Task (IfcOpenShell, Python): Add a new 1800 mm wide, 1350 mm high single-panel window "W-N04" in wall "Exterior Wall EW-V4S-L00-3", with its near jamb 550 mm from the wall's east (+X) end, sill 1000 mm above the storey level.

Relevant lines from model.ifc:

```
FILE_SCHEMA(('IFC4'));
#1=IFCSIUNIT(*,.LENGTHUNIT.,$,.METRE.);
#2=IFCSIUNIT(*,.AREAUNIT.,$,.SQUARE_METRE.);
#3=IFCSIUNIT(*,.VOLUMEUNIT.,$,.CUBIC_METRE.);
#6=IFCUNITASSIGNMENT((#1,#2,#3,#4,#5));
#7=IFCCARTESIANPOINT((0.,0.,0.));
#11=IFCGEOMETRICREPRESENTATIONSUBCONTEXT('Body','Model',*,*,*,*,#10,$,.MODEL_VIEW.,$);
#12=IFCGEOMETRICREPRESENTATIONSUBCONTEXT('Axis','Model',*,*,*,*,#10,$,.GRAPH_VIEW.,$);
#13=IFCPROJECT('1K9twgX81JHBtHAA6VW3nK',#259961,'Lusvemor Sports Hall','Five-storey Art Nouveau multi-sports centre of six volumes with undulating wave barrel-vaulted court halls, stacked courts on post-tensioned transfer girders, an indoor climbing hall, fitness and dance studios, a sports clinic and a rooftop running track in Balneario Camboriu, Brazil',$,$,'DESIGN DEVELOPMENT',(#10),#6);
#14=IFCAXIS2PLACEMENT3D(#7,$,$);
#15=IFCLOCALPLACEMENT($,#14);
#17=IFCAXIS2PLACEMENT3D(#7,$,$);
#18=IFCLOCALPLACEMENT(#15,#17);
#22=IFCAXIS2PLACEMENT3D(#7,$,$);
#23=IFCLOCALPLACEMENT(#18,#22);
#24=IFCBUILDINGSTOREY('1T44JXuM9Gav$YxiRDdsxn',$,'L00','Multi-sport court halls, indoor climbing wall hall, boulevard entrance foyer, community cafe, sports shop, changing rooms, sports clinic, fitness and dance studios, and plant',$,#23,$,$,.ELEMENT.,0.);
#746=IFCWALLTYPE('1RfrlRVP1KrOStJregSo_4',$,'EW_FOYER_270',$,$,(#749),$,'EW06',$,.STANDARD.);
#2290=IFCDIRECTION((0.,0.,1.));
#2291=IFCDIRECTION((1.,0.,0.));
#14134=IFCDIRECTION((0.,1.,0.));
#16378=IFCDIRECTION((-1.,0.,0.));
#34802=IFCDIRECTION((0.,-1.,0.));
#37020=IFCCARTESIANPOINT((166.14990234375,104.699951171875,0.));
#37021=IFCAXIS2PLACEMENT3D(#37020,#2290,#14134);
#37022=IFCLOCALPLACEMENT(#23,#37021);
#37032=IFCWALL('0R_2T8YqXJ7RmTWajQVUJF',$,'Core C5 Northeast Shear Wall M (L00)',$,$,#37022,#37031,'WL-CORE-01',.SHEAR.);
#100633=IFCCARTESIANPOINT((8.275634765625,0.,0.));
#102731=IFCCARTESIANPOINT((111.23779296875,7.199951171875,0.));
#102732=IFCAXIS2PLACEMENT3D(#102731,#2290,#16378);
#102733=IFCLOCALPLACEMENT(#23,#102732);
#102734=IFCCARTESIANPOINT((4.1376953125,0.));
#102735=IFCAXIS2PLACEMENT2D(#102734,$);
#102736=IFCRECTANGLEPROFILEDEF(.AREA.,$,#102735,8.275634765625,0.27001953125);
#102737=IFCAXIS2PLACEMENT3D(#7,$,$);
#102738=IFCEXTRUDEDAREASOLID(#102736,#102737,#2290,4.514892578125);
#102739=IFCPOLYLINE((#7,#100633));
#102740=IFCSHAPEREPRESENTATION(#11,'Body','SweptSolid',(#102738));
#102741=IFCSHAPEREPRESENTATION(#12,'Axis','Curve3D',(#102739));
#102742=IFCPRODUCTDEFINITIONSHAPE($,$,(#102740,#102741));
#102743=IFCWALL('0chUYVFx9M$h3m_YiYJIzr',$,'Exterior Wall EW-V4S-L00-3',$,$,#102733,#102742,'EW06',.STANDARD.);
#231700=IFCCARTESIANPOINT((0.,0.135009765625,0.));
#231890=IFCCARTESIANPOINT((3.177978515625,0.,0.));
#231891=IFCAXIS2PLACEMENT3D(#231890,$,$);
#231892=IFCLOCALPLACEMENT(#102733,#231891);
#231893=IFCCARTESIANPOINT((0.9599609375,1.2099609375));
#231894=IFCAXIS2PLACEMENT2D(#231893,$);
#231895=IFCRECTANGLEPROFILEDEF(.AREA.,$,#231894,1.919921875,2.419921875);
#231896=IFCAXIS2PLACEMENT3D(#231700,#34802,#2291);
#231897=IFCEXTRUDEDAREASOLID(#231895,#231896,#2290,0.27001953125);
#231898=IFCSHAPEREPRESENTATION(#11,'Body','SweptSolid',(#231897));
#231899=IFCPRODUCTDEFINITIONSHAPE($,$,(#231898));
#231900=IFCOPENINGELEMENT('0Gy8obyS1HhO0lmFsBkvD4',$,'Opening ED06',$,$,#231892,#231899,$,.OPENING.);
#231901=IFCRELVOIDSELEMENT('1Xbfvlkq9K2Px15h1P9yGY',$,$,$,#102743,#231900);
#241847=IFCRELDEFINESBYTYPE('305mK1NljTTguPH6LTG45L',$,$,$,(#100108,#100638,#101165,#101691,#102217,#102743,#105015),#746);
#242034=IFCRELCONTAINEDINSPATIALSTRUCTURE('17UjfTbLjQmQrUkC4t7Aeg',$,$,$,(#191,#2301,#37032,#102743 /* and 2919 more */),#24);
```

```python
import numpy as np
import ifcopenshell
import ifcopenshell.api.feature
import ifcopenshell.api.geometry
import ifcopenshell.api.root
import ifcopenshell.api.spatial
import ifcopenshell.geom
import ifcopenshell.util.element
import ifcopenshell.util.placement
import ifcopenshell.util.representation
import ifcopenshell.util.shape
import ifcopenshell.util.unit

model = ifcopenshell.open("model.ifc")
unit_scale = ifcopenshell.util.unit.calculate_unit_scale(model)
settings = ifcopenshell.geom.settings()


def volume(element):
    """Net volume in cubic metres, openings subtracted."""
    shape = ifcopenshell.geom.create_shape(settings, element)
    return ifcopenshell.util.shape.get_volume(shape.geometry)


wall = model.by_id(102743)
storey = ifcopenshell.util.element.get_container(wall, ifc_class="IfcBuildingStorey")
context = ifcopenshell.util.representation.get_context(model, "Model", "Body", "MODEL_VIEW")
before = volume(wall)

width, height, from_end, sill = 1.8, 1.35, 0.55, 1  # metres

# The wall runs along its own X axis, and the end named is its -X end.
wall_shape = ifcopenshell.geom.create_shape(settings, wall)
x, y, z = ifcopenshell.util.shape.get_vertices(wall_shape.geometry).T
start = x.min() + from_end
face, thickness = float(y.min()), float(y.max() - y.min())
wall_matrix = ifcopenshell.util.placement.get_local_placement(wall.ObjectPlacement)
level = ifcopenshell.util.placement.get_local_placement(storey.ObjectPlacement)[2, 3]


def in_wall(x, y):
    """Placement at x, y metres in the wall's axes, at sill height."""
    matrix = wall_matrix.copy()
    matrix[:, 3] = wall_matrix @ np.array([x / unit_scale, y / unit_scale, 0.0, 1.0])
    matrix[2, 3] = level + sill / unit_scale
    return matrix


# Opening: a box that overshoots both wall faces by 50 mm.
opening = ifcopenshell.api.root.create_entity(model, ifc_class="IfcOpeningElement", predefined_type="OPENING")
box = ifcopenshell.api.geometry.add_wall_representation(
    model, context=context, length=width, height=height, thickness=thickness + 0.1
)
ifcopenshell.api.geometry.assign_representation(model, product=opening, representation=box)
ifcopenshell.api.geometry.edit_object_placement(model, product=opening, matrix=in_wall(start, face - 0.05), is_si=False)
ifcopenshell.api.feature.add_feature(model, feature=opening, element=wall)

window = ifcopenshell.api.root.create_entity(model, ifc_class="IfcWindow", name="W-N04", predefined_type="WINDOW")
window.OverallWidth, window.OverallHeight = width / unit_scale, height / unit_scale
window.PartitioningType = "SINGLE_PANEL"
body = ifcopenshell.api.geometry.add_window_representation(
    model,
    context=context,
    overall_width=window.OverallWidth,
    overall_height=window.OverallHeight,
    partition_type="SINGLE_PANEL",
)
ifcopenshell.api.geometry.assign_representation(model, product=window, representation=body)
ifcopenshell.api.spatial.assign_container(model, products=[window], relating_structure=storey)
ifcopenshell.api.feature.add_filling(model, opening=opening, element=window)

# Centre the window in the wall's thickness.
ifcopenshell.api.geometry.edit_object_placement(model, product=window, matrix=in_wall(start, face), is_si=False)
window_shape = ifcopenshell.geom.create_shape(settings, window)
depth = ifcopenshell.util.shape.get_vertices(window_shape.geometry)[:, 1]
offset = face + thickness / 2 - (depth.min() + depth.max()) / 2
ifcopenshell.api.geometry.edit_object_placement(model, product=window, matrix=in_wall(start, offset), is_si=False)

after = volume(wall)

print(f"wall volume {before:.3f} -> {after:.3f} m3")

model.write("model_edited.ifc")
```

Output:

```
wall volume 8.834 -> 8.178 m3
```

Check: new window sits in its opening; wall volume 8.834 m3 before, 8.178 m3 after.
